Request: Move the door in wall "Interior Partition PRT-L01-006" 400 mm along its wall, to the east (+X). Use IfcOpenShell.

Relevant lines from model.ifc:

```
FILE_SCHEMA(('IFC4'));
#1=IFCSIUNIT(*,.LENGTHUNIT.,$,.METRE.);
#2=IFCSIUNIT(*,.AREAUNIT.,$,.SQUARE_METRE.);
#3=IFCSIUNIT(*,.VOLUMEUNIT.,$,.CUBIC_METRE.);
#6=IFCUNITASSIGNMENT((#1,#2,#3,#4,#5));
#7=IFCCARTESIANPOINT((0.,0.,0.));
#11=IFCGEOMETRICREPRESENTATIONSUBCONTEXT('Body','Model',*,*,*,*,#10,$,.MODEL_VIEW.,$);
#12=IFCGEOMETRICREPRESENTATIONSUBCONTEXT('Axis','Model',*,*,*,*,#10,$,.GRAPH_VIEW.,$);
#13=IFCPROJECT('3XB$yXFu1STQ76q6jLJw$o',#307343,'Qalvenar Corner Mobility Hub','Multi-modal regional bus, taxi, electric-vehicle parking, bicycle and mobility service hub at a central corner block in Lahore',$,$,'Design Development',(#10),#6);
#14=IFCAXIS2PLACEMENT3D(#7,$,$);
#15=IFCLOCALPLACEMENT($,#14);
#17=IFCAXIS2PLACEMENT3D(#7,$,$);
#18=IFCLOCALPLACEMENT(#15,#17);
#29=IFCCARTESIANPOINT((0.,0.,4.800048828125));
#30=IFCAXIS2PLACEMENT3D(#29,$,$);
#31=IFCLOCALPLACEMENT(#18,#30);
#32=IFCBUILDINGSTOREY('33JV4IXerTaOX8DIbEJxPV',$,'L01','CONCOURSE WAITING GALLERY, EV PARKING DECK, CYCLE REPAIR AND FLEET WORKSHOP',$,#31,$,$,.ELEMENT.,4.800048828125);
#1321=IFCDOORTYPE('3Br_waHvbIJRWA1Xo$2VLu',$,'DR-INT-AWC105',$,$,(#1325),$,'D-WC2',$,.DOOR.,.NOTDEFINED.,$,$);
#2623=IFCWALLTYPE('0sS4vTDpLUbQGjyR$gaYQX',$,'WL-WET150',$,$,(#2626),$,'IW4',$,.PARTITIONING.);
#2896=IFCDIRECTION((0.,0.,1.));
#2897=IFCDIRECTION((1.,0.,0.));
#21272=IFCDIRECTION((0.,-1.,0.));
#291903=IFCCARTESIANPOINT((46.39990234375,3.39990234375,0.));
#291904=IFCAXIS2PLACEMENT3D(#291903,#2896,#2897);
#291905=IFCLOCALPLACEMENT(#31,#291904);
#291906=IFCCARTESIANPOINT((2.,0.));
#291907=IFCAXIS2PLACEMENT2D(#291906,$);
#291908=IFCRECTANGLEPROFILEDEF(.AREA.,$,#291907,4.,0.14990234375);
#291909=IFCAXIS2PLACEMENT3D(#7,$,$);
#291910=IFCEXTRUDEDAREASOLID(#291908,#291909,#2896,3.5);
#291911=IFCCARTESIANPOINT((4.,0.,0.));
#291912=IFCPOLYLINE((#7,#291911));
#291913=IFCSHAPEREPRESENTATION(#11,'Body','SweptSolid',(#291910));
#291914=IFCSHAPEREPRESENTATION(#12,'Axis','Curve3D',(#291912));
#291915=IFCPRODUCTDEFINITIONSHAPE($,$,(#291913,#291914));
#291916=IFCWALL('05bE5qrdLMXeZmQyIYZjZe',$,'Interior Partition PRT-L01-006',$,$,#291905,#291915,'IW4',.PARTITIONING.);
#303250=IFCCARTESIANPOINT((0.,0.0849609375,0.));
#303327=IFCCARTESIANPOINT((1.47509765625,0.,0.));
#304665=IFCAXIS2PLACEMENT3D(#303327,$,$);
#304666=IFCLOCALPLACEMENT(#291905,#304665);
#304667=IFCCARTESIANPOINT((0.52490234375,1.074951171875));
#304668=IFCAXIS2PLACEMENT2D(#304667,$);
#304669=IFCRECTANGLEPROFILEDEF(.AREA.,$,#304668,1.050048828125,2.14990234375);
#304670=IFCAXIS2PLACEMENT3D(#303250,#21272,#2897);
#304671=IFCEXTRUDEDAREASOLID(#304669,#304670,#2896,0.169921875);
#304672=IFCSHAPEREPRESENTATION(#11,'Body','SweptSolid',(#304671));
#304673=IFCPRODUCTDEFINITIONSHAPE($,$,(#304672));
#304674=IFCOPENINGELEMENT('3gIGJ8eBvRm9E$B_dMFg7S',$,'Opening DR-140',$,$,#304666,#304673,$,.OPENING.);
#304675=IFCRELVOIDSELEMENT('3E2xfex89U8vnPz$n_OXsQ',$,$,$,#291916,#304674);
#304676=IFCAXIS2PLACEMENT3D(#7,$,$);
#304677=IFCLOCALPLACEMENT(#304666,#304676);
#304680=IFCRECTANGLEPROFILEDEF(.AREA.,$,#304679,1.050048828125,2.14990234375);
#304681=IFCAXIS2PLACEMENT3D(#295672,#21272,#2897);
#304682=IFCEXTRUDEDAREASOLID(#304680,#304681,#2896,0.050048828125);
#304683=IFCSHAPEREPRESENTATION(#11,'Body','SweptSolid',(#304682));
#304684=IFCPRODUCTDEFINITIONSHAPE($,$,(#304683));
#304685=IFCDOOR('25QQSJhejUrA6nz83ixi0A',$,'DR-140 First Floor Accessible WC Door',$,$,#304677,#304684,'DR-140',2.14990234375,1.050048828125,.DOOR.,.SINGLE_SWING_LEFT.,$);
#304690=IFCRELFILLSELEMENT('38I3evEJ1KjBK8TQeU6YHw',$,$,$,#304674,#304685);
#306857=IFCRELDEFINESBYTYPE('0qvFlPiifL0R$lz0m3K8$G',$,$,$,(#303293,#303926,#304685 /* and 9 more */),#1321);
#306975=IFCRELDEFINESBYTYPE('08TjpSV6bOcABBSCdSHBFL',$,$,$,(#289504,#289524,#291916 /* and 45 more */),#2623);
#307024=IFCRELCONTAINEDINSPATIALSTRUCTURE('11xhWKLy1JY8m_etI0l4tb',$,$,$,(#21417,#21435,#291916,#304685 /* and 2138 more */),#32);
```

```python
import ifcopenshell
import ifcopenshell.api.geometry
import ifcopenshell.util.placement

model = ifcopenshell.open("model.ifc")

door = model.by_id(304685)
opening = door.FillsVoids[0].RelatingOpeningElement
wall = opening.VoidsElements[0].RelatingBuildingElement

wall_matrix = ifcopenshell.util.placement.get_local_placement(wall.ObjectPlacement)
shift = wall_matrix[:3, 0] * 0.4
before = ifcopenshell.util.placement.get_local_placement(door.ObjectPlacement)[:3, 3].copy()

# The door is placed relative to its opening, so it follows when the opening moves.
matrix = ifcopenshell.util.placement.get_local_placement(opening.ObjectPlacement)
matrix[:3, 3] += shift
ifcopenshell.api.geometry.edit_object_placement(
    model, product=opening, matrix=matrix, is_si=False, should_transform_children=True
)

after = ifcopenshell.util.placement.get_local_placement(door.ObjectPlacement)[:3, 3]
print("door moved by", (after - before).round(3) + 0.0)

model.write("model-out.ifc")
```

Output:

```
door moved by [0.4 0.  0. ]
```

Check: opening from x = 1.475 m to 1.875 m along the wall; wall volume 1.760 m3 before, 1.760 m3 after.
